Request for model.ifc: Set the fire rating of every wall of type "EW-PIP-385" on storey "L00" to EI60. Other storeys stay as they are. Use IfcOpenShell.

First a look at what the model holds.

```python
import ifcopenshell
import ifcopenshell.util.element

model = ifcopenshell.open("model.ifc")
print(model.schema)
storey = next(s for s in model.by_type("IfcBuildingStorey") if s.Name == "L00")
walls = [e for e in ifcopenshell.util.element.get_decomposition(storey) if e.is_a("IfcWall")]
seen = {}
for e in walls:
    element_type = ifcopenshell.util.element.get_type(e)
    key = (element_type.Name if element_type != e and element_type else None, ifcopenshell.util.element.get_pset(e, "Pset_WallCommon", "FireRating"))
    seen[key] = seen.get(key, 0) + 1
for (name, value), count in sorted(seen.items(), key=str):
    print(count, "x", name, "|", value)
```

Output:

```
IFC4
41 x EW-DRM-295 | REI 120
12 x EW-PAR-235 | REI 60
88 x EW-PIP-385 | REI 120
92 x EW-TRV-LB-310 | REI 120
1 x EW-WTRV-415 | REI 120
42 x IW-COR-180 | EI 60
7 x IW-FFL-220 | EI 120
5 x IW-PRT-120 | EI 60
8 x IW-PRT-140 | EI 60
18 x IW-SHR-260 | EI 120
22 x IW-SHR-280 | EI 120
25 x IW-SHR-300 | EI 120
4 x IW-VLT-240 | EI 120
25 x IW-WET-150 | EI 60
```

```python
import ifcopenshell
import ifcopenshell.api.pset
import ifcopenshell.util.element

model = ifcopenshell.open("model.ifc")

storey = next(s for s in model.by_type("IfcBuildingStorey") if s.Name == "L00")
walls = [e for e in ifcopenshell.util.element.get_decomposition(storey) if e.is_a("IfcWall")]

count = 0
for e in walls:
    element_type = ifcopenshell.util.element.get_type(e)
    if element_type in (None, e) or element_type.Name != "EW-PIP-385":
        continue
    # add_pset returns the element's existing set when there is one.
    pset = ifcopenshell.api.pset.add_pset(model, product=e, name="Pset_WallCommon")
    ifcopenshell.api.pset.edit_pset(model, pset=pset, properties={"FireRating": "EI60"})
    count += 1

print(count, "walls updated")

model.write("model-out.ifc")
```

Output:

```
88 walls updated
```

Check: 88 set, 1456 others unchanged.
